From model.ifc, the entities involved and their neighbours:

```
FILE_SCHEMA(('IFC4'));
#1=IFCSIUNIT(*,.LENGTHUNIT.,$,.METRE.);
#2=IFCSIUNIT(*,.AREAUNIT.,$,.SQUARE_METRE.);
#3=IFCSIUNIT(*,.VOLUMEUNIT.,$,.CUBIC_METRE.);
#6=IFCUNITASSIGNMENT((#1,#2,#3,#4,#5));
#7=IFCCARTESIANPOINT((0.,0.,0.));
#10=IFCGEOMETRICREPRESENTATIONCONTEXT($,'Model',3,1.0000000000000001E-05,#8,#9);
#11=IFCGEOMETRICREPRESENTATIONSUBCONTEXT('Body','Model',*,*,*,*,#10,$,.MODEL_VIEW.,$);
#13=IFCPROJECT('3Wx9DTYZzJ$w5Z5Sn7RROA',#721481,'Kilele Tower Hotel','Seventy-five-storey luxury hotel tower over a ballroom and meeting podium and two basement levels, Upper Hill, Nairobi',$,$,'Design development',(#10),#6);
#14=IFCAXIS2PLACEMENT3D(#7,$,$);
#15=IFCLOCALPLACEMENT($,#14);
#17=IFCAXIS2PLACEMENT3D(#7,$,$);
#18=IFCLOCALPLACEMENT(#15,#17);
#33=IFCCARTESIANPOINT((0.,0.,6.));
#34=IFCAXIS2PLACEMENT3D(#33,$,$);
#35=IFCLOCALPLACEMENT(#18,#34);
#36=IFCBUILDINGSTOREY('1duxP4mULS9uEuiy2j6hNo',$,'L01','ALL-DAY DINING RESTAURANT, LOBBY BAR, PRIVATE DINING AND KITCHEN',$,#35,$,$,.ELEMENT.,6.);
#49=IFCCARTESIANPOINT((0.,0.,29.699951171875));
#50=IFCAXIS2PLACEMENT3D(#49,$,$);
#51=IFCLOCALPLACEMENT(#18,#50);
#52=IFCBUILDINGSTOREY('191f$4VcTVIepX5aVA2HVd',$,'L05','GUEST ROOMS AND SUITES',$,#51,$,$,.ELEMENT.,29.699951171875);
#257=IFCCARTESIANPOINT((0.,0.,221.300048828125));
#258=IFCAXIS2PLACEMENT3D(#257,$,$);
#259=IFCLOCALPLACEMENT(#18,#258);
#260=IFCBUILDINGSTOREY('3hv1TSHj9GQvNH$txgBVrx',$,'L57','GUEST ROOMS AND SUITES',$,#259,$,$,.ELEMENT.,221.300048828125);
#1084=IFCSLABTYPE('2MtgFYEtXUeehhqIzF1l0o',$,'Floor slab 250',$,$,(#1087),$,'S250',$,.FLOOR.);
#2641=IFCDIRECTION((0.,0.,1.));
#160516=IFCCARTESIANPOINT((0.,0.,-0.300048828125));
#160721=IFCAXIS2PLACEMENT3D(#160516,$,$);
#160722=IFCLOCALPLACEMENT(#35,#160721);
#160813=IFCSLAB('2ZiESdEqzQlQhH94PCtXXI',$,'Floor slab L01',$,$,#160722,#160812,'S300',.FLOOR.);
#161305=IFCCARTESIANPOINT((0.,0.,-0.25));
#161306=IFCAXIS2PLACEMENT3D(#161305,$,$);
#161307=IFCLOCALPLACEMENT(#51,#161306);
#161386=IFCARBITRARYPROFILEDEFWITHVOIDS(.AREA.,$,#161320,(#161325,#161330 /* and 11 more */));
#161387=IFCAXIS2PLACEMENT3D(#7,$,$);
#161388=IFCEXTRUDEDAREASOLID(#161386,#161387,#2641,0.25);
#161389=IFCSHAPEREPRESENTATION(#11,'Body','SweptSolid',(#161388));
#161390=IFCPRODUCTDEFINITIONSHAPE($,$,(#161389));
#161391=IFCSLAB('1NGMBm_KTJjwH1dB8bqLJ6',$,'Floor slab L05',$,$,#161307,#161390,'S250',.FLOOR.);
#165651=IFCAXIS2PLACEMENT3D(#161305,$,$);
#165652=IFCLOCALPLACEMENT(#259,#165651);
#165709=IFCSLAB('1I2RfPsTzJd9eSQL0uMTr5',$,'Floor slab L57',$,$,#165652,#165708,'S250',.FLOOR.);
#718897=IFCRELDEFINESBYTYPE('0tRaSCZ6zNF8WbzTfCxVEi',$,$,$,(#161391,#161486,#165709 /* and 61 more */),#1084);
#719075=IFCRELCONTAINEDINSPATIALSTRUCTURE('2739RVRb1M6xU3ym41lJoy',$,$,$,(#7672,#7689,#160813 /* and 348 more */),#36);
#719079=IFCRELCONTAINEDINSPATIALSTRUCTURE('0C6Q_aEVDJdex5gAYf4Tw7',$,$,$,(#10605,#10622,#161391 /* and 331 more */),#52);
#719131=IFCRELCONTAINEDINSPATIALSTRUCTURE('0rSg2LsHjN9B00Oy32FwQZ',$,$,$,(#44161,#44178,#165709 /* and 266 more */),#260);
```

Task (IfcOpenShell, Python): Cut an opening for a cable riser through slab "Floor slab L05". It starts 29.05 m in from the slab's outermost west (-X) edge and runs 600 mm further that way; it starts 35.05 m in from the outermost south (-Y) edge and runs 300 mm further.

```python
import numpy as np
import ifcopenshell
import ifcopenshell.api.feature
import ifcopenshell.api.geometry
import ifcopenshell.api.root
import ifcopenshell.geom
import ifcopenshell.util.placement
import ifcopenshell.util.representation
import ifcopenshell.util.shape
import ifcopenshell.util.unit

model = ifcopenshell.open("model.ifc")
unit_scale = ifcopenshell.util.unit.calculate_unit_scale(model)
settings = ifcopenshell.geom.settings()


def volume(element):
    """Net volume in cubic metres, openings subtracted."""
    shape = ifcopenshell.geom.create_shape(settings, element)
    return ifcopenshell.util.shape.get_volume(shape.geometry)


slab = model.by_guid("1NGMBm_KTJjwH1dB8bqLJ6")
before = volume(slab)

# Extent in the slab's own axes, in metres. The edges named are its -X and -Y sides.
slab_shape = ifcopenshell.geom.create_shape(settings, slab)
vertices = ifcopenshell.util.shape.get_vertices(slab_shape.geometry)
x_min, y_min, bottom = vertices.min(axis=0)
top = vertices[:, 2].max()

opening = ifcopenshell.api.root.create_entity(model, ifc_class="IfcOpeningElement", name="Cable riser opening", predefined_type="OPENING")
context = ifcopenshell.util.representation.get_context(model, "Model", "Body", "MODEL_VIEW")
width, depth = 0.6, 0.3
outline = [(0.0, 0.0), (width, 0.0), (width, depth), (0.0, depth), (0.0, 0.0)]
# Overshoot both faces by 50 mm so the cut is clean.
shape = ifcopenshell.api.geometry.add_slab_representation(
    model, context=context, depth=top - bottom + 0.1, polyline=outline
)
ifcopenshell.api.geometry.assign_representation(model, product=opening, representation=shape)

matrix = ifcopenshell.util.placement.get_local_placement(slab.ObjectPlacement)
matrix[:, 3] = matrix @ np.append(np.array([x_min + 29.05, y_min + 35.05, bottom - 0.05]) / unit_scale, 1.0)
ifcopenshell.api.geometry.edit_object_placement(model, product=opening, matrix=matrix, is_si=False)
ifcopenshell.api.feature.add_feature(model, feature=opening, element=slab)

after = volume(slab)

print(f"slab volume {before:.3f} -> {after:.3f} m3")

model.write("model_updated.ifc")
```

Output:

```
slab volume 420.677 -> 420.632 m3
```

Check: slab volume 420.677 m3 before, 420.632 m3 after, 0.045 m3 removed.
